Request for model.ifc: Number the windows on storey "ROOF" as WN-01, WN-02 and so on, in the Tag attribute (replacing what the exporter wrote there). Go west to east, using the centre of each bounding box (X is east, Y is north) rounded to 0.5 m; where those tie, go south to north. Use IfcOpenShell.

First a look at what the model holds.

```python
import ifcopenshell
import ifcopenshell.util.element
import ifcopenshell.util.placement

model = ifcopenshell.open("model.ifc")
print(model.schema)
storey = next(s for s in model.by_type("IfcBuildingStorey") if s.Name == "ROOF")
windows = [e for e in ifcopenshell.util.element.get_decomposition(storey) if e.is_a("IfcWindow")]
for e in sorted(windows, key=lambda e: e.id()):
    origin = ifcopenshell.util.placement.get_local_placement(e.ObjectPlacement)[:3, 3]
    print(e.id(), e.Tag, e.Name, origin.round(2) + 0.0, sep=" | ")
```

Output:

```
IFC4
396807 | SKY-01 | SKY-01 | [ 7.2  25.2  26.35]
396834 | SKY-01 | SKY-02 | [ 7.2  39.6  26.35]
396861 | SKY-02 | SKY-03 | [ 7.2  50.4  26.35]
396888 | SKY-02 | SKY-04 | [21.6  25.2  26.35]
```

```python
import ifcopenshell
import ifcopenshell.geom
import ifcopenshell.util.element
import ifcopenshell.util.shape

model = ifcopenshell.open("model.ifc")
settings = ifcopenshell.geom.settings()
settings.set("use-world-coords", True)


def centre(element):
    shape = ifcopenshell.geom.create_shape(settings, element)
    return ifcopenshell.util.shape.get_bbox_centroid(shape.geometry)


storey = next(s for s in model.by_type("IfcBuildingStorey") if s.Name == "ROOF")
windows = [e for e in ifcopenshell.util.element.get_decomposition(storey) if e.is_a("IfcWindow")]

# Insertion points can sit at a corner or the storey origin, so sort by the geometry (in metres).
centres = {e: centre(e) for e in windows}
windows.sort(key=lambda e: (round(centres[e][0] / 0.5), centres[e][1]))

for i, e in enumerate(windows, start=1):
    number = f"WN-{i:02d}"
    e.Tag = number
    print(e.id(), number)

model.write("model_updated.ifc")
```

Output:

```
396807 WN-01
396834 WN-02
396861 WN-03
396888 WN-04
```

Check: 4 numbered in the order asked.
